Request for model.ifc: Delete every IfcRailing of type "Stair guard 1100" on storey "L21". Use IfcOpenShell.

First a look at what the model holds.

```python
import ifcopenshell
import ifcopenshell.util.element

model = ifcopenshell.open("model.ifc")
print(model.schema)
storey = next(s for s in model.by_type("IfcBuildingStorey") if s.Name == "L21")
railings = [e for e in ifcopenshell.util.element.get_decomposition(storey) if e.is_a("IfcRailing")]
seen = {}
for e in railings:
    element_type = ifcopenshell.util.element.get_type(e)
    name = element_type.Name if element_type not in (None, e) else None
    seen[name] = seen.get(name, 0) + 1
for name, count in sorted(seen.items(), key=str):
    print(count, "x", name)
```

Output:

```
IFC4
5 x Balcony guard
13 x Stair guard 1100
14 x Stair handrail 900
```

```python
import ifcopenshell
import ifcopenshell.api.root
import ifcopenshell.util.element

model = ifcopenshell.open("model.ifc")

storey = next(s for s in model.by_type("IfcBuildingStorey") if s.Name == "L21")
railings = [e for e in ifcopenshell.util.element.get_decomposition(storey) if e.is_a("IfcRailing")]
targets = [e for e in railings if (t := ifcopenshell.util.element.get_type(e)) not in (None, e) and t.Name == "Stair guard 1100"]

for e in targets:
    ifcopenshell.api.root.remove_product(model, product=e)
print(len(targets), "removed")

model.write("model_updated.ifc")
```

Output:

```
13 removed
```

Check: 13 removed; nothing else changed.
